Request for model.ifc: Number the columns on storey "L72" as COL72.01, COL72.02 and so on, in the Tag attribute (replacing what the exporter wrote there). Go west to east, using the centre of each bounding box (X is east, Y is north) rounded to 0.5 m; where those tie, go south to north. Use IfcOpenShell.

First a look at what the model holds.

```python
import ifcopenshell
import ifcopenshell.util.element
import ifcopenshell.util.placement

model = ifcopenshell.open("model.ifc")
print(model.schema)
storey = next(s for s in model.by_type("IfcBuildingStorey") if s.Name == "L72")
columns = [e for e in ifcopenshell.util.element.get_decomposition(storey) if e.is_a("IfcColumn")]
for e in sorted(columns, key=lambda e: e.id()):
    origin = ifcopenshell.util.placement.get_local_placement(e.ObjectPlacement)[:3, 3]
    print(e.id(), e.Tag, e.Name, origin.round(2) + 0.0, sep=" | ")
```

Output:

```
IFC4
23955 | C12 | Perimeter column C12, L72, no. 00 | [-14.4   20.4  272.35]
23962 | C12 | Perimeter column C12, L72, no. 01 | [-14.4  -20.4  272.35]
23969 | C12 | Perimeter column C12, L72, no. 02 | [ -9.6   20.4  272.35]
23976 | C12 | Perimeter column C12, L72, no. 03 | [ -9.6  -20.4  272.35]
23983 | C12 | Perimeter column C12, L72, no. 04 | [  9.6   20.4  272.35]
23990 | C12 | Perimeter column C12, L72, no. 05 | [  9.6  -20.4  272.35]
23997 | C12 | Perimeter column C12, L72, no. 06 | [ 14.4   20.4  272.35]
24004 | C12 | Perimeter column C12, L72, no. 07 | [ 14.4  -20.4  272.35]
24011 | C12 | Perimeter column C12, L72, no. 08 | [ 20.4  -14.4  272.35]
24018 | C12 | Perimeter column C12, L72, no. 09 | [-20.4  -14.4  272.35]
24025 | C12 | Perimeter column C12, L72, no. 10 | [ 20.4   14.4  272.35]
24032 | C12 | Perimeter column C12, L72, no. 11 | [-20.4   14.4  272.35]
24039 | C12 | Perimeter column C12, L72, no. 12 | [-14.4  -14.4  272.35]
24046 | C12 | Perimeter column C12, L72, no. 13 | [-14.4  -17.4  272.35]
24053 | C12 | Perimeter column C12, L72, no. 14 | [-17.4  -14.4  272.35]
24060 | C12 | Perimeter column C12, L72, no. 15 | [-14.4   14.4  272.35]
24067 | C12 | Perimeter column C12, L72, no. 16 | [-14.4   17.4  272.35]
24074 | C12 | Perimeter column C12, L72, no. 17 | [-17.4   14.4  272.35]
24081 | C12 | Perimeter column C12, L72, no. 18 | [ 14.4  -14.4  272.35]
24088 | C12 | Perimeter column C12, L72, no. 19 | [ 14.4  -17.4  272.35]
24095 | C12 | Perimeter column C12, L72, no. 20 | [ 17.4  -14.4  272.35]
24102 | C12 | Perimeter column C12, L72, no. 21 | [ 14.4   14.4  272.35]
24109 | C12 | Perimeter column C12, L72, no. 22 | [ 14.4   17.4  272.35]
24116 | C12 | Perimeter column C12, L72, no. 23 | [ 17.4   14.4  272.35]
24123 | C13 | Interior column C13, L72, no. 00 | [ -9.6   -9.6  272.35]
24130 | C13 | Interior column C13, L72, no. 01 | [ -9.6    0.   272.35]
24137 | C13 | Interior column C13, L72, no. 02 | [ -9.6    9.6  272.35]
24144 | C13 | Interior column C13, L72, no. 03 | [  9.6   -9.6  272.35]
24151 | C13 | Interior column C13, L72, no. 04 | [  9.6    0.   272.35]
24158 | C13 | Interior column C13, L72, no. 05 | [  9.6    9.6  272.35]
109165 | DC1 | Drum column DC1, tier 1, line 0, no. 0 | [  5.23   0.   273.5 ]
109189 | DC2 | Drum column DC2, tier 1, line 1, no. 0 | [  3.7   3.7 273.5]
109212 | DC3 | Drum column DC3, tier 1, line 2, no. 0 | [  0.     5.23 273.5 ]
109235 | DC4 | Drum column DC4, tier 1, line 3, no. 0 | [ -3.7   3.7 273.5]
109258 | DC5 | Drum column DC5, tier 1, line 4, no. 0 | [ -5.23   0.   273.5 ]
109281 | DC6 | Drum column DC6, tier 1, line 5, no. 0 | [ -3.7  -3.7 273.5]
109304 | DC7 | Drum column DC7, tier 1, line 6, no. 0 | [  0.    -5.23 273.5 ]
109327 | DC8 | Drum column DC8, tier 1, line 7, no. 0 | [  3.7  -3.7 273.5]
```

```python
import ifcopenshell
import ifcopenshell.geom
import ifcopenshell.util.element
import ifcopenshell.util.shape

model = ifcopenshell.open("model.ifc")
settings = ifcopenshell.geom.settings()
settings.set("use-world-coords", True)


def centre(element):
    shape = ifcopenshell.geom.create_shape(settings, element)
    return ifcopenshell.util.shape.get_bbox_centroid(shape.geometry)


storey = next(s for s in model.by_type("IfcBuildingStorey") if s.Name == "L72")
columns = [e for e in ifcopenshell.util.element.get_decomposition(storey) if e.is_a("IfcColumn")]

# Insertion points can sit at a corner or the storey origin, so sort by the geometry (in metres).
centres = {e: centre(e) for e in columns}
columns.sort(key=lambda e: (round(centres[e][0] / 0.5), centres[e][1]))

for i, e in enumerate(columns, start=1):
    number = f"COL72.{i:02d}"
    e.Tag = number
    print(e.id(), number)

model.write("model-out.ifc")
```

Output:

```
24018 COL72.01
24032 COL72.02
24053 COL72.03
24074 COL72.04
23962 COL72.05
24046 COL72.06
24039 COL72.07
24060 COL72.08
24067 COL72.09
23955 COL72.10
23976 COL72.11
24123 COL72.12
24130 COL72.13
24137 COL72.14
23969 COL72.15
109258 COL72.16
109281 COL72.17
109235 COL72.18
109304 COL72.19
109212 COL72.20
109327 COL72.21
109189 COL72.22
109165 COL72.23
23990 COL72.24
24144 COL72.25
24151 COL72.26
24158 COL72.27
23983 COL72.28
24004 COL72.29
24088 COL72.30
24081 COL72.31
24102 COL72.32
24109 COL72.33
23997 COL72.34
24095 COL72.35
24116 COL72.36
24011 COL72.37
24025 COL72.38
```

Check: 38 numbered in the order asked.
